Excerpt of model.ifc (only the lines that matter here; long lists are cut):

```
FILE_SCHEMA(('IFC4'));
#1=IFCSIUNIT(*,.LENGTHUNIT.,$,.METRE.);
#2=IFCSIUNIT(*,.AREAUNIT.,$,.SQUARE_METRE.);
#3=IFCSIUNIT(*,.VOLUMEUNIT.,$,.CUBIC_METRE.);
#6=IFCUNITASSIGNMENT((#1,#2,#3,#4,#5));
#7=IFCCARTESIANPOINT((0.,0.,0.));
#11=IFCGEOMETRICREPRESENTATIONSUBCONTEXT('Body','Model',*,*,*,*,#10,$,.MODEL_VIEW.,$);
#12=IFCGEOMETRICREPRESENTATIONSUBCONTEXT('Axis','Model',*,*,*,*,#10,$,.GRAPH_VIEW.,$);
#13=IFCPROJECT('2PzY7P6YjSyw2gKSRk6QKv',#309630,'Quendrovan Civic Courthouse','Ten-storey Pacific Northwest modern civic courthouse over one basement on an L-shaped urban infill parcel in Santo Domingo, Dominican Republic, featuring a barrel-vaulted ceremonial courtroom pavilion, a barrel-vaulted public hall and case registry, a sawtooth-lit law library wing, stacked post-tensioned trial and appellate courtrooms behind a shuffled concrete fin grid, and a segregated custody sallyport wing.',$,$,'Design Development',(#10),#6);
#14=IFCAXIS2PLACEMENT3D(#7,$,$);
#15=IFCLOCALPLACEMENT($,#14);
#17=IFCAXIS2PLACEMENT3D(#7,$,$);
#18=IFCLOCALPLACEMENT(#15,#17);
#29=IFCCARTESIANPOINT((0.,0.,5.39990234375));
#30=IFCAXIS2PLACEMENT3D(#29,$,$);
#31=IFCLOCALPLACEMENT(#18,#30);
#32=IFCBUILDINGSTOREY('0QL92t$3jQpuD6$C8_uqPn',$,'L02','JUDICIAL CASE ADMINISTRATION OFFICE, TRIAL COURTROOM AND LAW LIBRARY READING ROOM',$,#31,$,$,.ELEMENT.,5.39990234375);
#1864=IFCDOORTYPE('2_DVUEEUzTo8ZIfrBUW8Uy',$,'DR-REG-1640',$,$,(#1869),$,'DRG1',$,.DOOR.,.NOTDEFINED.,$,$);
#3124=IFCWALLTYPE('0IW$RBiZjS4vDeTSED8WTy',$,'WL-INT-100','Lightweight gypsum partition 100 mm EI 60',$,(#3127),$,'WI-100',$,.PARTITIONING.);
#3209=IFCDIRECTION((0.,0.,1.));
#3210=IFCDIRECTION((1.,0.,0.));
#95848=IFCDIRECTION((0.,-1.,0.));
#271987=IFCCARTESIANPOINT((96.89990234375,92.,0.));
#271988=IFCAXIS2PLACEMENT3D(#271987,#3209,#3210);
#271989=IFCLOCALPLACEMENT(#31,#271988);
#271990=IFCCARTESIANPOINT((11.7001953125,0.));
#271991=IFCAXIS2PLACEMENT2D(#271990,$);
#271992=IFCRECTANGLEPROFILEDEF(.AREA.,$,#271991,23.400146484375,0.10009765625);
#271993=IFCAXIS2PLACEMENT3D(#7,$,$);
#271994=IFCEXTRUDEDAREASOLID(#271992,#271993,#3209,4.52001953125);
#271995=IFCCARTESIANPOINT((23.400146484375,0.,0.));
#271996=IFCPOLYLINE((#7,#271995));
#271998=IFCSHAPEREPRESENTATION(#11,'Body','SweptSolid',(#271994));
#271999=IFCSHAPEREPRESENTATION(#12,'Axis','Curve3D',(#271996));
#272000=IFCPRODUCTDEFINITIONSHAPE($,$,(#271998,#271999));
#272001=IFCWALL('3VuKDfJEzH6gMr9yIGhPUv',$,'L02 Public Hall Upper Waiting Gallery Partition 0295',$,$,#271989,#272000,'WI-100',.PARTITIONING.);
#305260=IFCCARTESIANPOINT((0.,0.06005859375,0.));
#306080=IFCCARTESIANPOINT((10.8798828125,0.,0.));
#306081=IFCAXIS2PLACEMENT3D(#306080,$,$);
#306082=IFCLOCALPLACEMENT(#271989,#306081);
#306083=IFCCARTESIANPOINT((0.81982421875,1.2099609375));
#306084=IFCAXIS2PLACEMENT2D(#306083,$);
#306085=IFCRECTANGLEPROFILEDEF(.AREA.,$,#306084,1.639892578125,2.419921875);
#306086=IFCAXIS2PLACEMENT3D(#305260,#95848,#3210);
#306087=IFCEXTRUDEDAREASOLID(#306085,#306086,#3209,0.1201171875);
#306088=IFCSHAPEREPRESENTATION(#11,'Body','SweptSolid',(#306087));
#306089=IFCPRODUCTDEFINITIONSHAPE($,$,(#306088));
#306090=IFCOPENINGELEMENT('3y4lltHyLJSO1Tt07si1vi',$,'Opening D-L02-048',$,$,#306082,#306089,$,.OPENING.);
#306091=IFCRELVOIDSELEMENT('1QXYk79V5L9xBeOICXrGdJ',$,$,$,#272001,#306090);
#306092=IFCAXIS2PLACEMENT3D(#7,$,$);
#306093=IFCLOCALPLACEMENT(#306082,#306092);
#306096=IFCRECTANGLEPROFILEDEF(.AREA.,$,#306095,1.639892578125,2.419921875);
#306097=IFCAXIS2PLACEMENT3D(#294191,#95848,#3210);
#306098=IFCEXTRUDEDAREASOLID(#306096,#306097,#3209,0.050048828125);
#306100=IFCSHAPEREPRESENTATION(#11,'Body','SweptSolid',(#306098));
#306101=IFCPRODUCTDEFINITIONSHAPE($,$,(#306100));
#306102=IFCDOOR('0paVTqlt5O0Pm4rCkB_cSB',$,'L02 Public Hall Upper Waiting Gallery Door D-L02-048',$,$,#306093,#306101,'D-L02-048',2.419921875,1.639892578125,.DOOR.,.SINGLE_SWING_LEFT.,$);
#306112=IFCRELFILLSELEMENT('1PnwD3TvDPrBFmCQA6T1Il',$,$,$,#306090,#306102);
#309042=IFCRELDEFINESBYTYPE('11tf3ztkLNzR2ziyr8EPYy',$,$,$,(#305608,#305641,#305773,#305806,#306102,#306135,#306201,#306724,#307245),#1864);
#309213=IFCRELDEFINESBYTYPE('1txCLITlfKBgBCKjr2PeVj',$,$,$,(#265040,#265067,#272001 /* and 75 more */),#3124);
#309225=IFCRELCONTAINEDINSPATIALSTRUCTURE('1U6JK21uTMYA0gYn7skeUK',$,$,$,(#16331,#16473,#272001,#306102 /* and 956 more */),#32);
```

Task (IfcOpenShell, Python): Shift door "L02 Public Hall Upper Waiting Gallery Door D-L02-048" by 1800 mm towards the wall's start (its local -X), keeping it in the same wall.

```python
import ifcopenshell
import ifcopenshell.api.geometry
import ifcopenshell.util.placement
import ifcopenshell.util.unit

model = ifcopenshell.open("model.ifc")
unit_scale = ifcopenshell.util.unit.calculate_unit_scale(model)

door = model.by_guid("0paVTqlt5O0Pm4rCkB_cSB")
opening = door.FillsVoids[0].RelatingOpeningElement
wall = opening.VoidsElements[0].RelatingBuildingElement

wall_matrix = ifcopenshell.util.placement.get_local_placement(wall.ObjectPlacement)
shift = wall_matrix[:3, 0] * -1.8 / unit_scale
before = ifcopenshell.util.placement.get_local_placement(door.ObjectPlacement)[:3, 3].copy()

# The door is placed relative to its opening, so it follows when the opening moves.
matrix = ifcopenshell.util.placement.get_local_placement(opening.ObjectPlacement)
matrix[:3, 3] += shift
ifcopenshell.api.geometry.edit_object_placement(
    model, product=opening, matrix=matrix, is_si=False, should_transform_children=True
)

after = ifcopenshell.util.placement.get_local_placement(door.ObjectPlacement)[:3, 3]
print("door moved by", (after - before).round(3) + 0.0)

model.write("model_rev.ifc")
```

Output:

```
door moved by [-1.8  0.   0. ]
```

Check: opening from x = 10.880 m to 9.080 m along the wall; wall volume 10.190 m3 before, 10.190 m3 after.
